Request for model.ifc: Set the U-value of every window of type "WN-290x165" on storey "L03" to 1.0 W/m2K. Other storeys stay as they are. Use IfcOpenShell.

First a look at what the model holds.

```python
import ifcopenshell
import ifcopenshell.util.element

model = ifcopenshell.open("model.ifc")
print(model.schema)
storey = next(s for s in model.by_type("IfcBuildingStorey") if s.Name == "L03")
windows = [e for e in ifcopenshell.util.element.get_decomposition(storey) if e.is_a("IfcWindow")]
seen = {}
for e in windows:
    element_type = ifcopenshell.util.element.get_type(e)
    key = (element_type.Name if element_type != e and element_type else None, ifcopenshell.util.element.get_pset(e, "Pset_WindowCommon", "ThermalTransmittance"))
    seen[key] = seen.get(key, 0) + 1
for (name, value), count in sorted(seen.items(), key=str):
    print(count, "x", name, "|", value)
```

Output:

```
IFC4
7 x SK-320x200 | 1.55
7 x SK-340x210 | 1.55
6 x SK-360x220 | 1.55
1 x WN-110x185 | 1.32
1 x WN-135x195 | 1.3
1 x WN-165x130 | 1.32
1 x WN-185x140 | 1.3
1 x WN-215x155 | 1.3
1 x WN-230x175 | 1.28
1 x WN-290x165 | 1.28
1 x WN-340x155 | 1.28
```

```python
import ifcopenshell
import ifcopenshell.api.pset
import ifcopenshell.util.element

model = ifcopenshell.open("model.ifc")

storey = next(s for s in model.by_type("IfcBuildingStorey") if s.Name == "L03")
windows = [e for e in ifcopenshell.util.element.get_decomposition(storey) if e.is_a("IfcWindow")]

count = 0
for e in windows:
    element_type = ifcopenshell.util.element.get_type(e)
    if element_type in (None, e) or element_type.Name != "WN-290x165":
        continue
    # add_pset returns the element's existing set when there is one.
    pset = ifcopenshell.api.pset.add_pset(model, product=e, name="Pset_WindowCommon")
    ifcopenshell.api.pset.edit_pset(model, pset=pset, properties={"ThermalTransmittance": 1.0})
    count += 1

print(count, "windows updated")

model.write("model_v2.ifc")
```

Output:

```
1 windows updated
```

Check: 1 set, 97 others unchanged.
